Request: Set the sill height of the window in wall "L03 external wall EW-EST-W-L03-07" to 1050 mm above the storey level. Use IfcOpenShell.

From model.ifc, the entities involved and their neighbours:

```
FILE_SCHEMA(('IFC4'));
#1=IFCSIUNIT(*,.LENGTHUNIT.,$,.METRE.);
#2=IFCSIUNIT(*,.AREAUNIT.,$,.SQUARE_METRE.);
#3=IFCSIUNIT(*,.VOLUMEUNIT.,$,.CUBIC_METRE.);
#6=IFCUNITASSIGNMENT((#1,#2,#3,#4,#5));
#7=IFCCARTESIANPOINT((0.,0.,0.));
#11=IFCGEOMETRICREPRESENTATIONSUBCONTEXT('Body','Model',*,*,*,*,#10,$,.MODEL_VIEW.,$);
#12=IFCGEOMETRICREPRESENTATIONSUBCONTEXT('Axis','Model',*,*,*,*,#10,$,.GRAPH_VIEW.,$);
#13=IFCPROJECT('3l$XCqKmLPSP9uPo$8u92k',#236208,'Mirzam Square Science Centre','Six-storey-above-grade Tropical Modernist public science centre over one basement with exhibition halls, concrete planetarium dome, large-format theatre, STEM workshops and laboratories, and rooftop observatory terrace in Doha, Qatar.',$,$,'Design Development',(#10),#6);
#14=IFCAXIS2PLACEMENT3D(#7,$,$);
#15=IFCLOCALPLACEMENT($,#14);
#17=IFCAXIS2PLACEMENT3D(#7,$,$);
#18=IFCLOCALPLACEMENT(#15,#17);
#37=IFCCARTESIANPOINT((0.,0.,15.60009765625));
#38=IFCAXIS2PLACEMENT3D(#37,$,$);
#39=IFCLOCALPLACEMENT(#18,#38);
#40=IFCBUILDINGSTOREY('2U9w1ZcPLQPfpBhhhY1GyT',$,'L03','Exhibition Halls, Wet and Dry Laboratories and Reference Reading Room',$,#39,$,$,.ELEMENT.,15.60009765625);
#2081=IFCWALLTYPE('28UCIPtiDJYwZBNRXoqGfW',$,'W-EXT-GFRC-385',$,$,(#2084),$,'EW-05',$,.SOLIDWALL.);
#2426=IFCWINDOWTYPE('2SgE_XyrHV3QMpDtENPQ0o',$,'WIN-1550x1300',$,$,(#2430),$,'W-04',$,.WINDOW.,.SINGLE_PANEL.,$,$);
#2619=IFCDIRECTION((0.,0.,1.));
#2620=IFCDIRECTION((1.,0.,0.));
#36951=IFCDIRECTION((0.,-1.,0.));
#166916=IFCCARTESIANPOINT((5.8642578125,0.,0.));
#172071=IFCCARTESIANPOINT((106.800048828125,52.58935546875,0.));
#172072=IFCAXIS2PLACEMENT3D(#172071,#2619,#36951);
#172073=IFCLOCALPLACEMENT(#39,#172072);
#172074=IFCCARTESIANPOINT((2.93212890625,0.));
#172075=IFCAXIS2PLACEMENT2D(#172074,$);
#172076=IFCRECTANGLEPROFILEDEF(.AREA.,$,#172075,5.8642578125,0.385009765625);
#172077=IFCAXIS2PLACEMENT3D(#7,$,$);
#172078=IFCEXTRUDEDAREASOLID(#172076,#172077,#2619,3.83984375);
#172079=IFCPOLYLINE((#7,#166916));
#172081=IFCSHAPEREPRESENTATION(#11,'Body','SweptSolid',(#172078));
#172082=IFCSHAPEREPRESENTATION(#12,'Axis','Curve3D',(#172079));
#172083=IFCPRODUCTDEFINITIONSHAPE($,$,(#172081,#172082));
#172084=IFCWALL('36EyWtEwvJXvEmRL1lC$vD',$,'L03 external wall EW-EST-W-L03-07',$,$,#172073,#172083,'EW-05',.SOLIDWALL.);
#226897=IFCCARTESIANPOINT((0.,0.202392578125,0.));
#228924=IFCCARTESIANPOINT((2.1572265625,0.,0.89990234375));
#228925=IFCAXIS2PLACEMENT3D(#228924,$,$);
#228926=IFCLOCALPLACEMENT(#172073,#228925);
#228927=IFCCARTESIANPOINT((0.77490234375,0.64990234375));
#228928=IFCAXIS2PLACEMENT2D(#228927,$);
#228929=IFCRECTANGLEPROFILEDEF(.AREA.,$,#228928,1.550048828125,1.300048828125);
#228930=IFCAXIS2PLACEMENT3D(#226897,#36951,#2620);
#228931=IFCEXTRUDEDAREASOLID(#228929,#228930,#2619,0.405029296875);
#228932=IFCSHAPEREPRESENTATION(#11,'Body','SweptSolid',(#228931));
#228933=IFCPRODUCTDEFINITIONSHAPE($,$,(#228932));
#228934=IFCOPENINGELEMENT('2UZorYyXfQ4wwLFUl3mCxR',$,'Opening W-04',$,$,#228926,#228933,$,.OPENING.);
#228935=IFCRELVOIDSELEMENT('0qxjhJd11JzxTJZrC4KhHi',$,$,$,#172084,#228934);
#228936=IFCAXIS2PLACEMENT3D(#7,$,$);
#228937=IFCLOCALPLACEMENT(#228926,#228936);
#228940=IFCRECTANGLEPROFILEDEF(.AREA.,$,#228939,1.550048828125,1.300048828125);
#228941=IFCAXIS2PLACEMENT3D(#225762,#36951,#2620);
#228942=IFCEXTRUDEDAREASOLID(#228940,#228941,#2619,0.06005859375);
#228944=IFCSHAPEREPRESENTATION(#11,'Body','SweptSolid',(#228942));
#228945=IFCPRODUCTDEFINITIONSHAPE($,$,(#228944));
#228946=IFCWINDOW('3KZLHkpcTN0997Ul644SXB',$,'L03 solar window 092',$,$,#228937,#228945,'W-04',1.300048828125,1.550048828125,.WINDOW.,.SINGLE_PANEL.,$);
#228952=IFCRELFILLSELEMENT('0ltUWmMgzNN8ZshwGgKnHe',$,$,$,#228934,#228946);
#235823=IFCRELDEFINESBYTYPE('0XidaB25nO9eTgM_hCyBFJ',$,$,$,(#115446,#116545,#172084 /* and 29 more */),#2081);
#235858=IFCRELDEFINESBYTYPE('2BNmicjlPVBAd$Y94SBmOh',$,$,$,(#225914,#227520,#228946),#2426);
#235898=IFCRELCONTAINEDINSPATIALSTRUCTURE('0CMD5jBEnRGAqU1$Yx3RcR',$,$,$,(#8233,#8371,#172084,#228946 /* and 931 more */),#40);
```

```python
import numpy as np
import ifcopenshell
import ifcopenshell.api.geometry
import ifcopenshell.geom
import ifcopenshell.util.element
import ifcopenshell.util.placement
import ifcopenshell.util.shape
import ifcopenshell.util.unit

model = ifcopenshell.open("model.ifc")
unit_scale = ifcopenshell.util.unit.calculate_unit_scale(model)

window = model.by_id(228946)
opening = window.FillsVoids[0].RelatingOpeningElement
storey = ifcopenshell.util.element.get_container(window, ifc_class="IfcBuildingStorey")
level = ifcopenshell.util.placement.get_local_placement(storey.ObjectPlacement)[2, 3]

# The opening's origin need not be at the sill, so measure its lowest point.
shape = ifcopenshell.geom.create_shape(ifcopenshell.geom.settings(), opening)
bottom = ifcopenshell.util.shape.get_shape_bottom_elevation(shape, shape.geometry) / unit_scale
dz = level + 1.05 - bottom

shift = np.array([0.0, 0.0, dz])
# The window is placed relative to its opening, so it follows when the opening moves.
matrix = ifcopenshell.util.placement.get_local_placement(opening.ObjectPlacement)
matrix[:3, 3] += shift
ifcopenshell.api.geometry.edit_object_placement(
    model, product=opening, matrix=matrix, is_si=False, should_transform_children=True
)

print(f"moved by {dz * unit_scale:+.3f} m")

model.write("model_updated.ifc")
```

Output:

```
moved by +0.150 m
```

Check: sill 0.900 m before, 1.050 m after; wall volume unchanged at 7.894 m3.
